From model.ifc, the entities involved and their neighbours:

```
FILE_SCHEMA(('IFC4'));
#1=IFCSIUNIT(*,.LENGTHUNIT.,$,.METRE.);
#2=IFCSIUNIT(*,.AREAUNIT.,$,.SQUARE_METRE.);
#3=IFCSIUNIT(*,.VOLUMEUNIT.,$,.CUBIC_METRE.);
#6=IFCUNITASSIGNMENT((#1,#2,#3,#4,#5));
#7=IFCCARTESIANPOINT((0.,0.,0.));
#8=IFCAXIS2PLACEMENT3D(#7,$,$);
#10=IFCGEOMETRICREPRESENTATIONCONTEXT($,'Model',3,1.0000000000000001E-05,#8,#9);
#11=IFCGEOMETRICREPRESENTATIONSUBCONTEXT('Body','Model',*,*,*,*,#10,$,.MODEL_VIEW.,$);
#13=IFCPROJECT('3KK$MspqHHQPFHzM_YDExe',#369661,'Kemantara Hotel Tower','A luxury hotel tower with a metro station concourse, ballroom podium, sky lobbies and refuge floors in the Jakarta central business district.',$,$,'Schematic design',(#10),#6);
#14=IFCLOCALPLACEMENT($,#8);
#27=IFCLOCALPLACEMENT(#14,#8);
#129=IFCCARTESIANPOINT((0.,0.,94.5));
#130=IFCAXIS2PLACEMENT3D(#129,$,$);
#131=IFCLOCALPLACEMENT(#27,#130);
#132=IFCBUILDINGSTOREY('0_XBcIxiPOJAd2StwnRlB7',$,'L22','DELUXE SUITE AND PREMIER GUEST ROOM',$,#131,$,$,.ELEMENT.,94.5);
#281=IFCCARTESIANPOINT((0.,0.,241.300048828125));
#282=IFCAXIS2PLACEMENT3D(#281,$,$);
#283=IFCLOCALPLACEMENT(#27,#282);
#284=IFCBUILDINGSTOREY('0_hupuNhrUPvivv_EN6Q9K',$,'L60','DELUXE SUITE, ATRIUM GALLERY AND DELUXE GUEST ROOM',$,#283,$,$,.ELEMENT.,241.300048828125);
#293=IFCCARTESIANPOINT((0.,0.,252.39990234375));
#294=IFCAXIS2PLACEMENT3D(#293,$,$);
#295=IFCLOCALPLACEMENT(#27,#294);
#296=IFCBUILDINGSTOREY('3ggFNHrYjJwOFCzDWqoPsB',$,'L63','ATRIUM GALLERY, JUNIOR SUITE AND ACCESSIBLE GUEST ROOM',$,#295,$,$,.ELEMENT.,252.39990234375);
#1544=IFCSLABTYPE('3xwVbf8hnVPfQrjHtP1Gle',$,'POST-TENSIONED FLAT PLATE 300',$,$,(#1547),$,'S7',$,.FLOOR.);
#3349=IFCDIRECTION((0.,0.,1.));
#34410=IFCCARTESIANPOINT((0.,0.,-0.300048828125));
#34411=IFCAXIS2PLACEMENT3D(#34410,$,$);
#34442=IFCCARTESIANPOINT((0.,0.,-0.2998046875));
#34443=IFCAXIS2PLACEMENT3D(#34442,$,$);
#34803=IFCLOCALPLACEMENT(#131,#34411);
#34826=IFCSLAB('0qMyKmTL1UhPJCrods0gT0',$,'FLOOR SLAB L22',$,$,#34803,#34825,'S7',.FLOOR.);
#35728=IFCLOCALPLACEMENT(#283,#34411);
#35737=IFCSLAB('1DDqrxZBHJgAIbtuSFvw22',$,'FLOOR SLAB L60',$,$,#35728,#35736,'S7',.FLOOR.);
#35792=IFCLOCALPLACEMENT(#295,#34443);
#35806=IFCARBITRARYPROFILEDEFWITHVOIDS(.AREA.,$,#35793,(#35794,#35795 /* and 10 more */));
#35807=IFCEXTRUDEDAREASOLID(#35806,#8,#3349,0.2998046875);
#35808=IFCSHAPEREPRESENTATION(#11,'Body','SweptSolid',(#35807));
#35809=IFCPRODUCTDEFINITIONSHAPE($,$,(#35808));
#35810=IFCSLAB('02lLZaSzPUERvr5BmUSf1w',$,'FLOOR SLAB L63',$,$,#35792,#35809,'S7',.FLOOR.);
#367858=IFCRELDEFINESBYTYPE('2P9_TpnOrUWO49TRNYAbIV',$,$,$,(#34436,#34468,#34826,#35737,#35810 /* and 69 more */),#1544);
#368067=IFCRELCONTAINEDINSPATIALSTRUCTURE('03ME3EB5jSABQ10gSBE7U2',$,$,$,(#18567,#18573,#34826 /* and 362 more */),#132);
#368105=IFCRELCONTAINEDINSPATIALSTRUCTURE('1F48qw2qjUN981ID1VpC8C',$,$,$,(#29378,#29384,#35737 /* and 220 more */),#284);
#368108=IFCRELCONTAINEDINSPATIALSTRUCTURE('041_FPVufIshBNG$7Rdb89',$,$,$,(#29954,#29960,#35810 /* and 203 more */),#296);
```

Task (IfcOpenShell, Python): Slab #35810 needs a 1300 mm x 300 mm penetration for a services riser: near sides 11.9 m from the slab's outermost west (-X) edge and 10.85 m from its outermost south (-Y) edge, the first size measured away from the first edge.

```python
import numpy as np
import ifcopenshell
import ifcopenshell.api.feature
import ifcopenshell.api.geometry
import ifcopenshell.api.root
import ifcopenshell.geom
import ifcopenshell.util.placement
import ifcopenshell.util.representation
import ifcopenshell.util.shape
import ifcopenshell.util.unit

model = ifcopenshell.open("model.ifc")
unit_scale = ifcopenshell.util.unit.calculate_unit_scale(model)
settings = ifcopenshell.geom.settings()


def volume(element):
    """Net volume in cubic metres, openings subtracted."""
    shape = ifcopenshell.geom.create_shape(settings, element)
    return ifcopenshell.util.shape.get_volume(shape.geometry)


slab = model.by_guid("02lLZaSzPUERvr5BmUSf1w")
before = volume(slab)

# Extent in the slab's own axes, in metres. The edges named are its -X and -Y sides.
slab_shape = ifcopenshell.geom.create_shape(settings, slab)
vertices = ifcopenshell.util.shape.get_vertices(slab_shape.geometry)
x_min, y_min, bottom = vertices.min(axis=0)
top = vertices[:, 2].max()

opening = ifcopenshell.api.root.create_entity(model, ifc_class="IfcOpeningElement", name="Services riser opening", predefined_type="OPENING")
context = ifcopenshell.util.representation.get_context(model, "Model", "Body", "MODEL_VIEW")
width, depth = 1.3, 0.3
outline = [(0.0, 0.0), (width, 0.0), (width, depth), (0.0, depth), (0.0, 0.0)]
# Overshoot both faces by 50 mm so the cut is clean.
shape = ifcopenshell.api.geometry.add_slab_representation(
    model, context=context, depth=top - bottom + 0.1, polyline=outline
)
ifcopenshell.api.geometry.assign_representation(model, product=opening, representation=shape)

matrix = ifcopenshell.util.placement.get_local_placement(slab.ObjectPlacement)
matrix[:, 3] = matrix @ np.append(np.array([x_min + 11.9, y_min + 10.85, bottom - 0.05]) / unit_scale, 1.0)
ifcopenshell.api.geometry.edit_object_placement(model, product=opening, matrix=matrix, is_si=False)
ifcopenshell.api.feature.add_feature(model, feature=opening, element=slab)

after = volume(slab)

print(f"slab volume {before:.3f} -> {after:.3f} m3")

model.write("model-out.ifc")
```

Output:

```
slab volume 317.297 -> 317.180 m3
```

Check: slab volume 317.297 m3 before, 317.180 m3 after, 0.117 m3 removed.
